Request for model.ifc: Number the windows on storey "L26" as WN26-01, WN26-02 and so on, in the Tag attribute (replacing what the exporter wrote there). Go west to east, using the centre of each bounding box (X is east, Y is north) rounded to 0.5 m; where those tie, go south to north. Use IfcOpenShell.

First a look at what the model holds.

```python
import ifcopenshell
import ifcopenshell.util.element
import ifcopenshell.util.placement

model = ifcopenshell.open("model.ifc")
print(model.schema)
storey = next(s for s in model.by_type("IfcBuildingStorey") if s.Name == "L26")
windows = [e for e in ifcopenshell.util.element.get_decomposition(storey) if e.is_a("IfcWindow")]
for e in sorted(windows, key=lambda e: e.id()):
    origin = ifcopenshell.util.placement.get_local_placement(e.ObjectPlacement)[:3, 3]
    print(e.id(), e.Tag, e.Name, origin.round(2) + 0.0, sep=" | ")
```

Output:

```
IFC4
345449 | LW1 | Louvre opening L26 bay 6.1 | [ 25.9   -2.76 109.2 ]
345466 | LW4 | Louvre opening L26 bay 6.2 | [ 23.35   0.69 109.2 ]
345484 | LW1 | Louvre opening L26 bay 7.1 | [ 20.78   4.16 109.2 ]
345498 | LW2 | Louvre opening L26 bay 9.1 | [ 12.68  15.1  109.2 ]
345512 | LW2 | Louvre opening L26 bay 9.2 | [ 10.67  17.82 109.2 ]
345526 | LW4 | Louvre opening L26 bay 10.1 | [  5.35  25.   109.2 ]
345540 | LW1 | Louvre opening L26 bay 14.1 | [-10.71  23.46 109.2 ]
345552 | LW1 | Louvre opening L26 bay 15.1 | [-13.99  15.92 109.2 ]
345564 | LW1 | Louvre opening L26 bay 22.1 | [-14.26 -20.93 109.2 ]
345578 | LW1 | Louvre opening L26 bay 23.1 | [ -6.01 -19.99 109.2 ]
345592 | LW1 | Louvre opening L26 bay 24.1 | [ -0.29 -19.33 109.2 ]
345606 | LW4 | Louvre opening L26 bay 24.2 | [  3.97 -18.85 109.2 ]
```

```python
import ifcopenshell
import ifcopenshell.geom
import ifcopenshell.util.element
import ifcopenshell.util.shape

model = ifcopenshell.open("model.ifc")
settings = ifcopenshell.geom.settings()
settings.set("use-world-coords", True)


def centre(element):
    shape = ifcopenshell.geom.create_shape(settings, element)
    return ifcopenshell.util.shape.get_bbox_centroid(shape.geometry)


storey = next(s for s in model.by_type("IfcBuildingStorey") if s.Name == "L26")
windows = [e for e in ifcopenshell.util.element.get_decomposition(storey) if e.is_a("IfcWindow")]

# Insertion points can sit at a corner or the storey origin, so sort by the geometry (in metres).
centres = {e: centre(e) for e in windows}
windows.sort(key=lambda e: (round(centres[e][0] / 0.5), centres[e][1]))

for i, e in enumerate(windows, start=1):
    number = f"WN26-{i:02d}"
    e.Tag = number
    print(e.id(), number)

model.write("model_rev.ifc")
```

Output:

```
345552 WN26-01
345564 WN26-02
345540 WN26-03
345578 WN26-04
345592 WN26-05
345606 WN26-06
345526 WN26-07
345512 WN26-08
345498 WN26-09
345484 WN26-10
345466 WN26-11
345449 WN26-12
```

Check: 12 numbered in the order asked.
